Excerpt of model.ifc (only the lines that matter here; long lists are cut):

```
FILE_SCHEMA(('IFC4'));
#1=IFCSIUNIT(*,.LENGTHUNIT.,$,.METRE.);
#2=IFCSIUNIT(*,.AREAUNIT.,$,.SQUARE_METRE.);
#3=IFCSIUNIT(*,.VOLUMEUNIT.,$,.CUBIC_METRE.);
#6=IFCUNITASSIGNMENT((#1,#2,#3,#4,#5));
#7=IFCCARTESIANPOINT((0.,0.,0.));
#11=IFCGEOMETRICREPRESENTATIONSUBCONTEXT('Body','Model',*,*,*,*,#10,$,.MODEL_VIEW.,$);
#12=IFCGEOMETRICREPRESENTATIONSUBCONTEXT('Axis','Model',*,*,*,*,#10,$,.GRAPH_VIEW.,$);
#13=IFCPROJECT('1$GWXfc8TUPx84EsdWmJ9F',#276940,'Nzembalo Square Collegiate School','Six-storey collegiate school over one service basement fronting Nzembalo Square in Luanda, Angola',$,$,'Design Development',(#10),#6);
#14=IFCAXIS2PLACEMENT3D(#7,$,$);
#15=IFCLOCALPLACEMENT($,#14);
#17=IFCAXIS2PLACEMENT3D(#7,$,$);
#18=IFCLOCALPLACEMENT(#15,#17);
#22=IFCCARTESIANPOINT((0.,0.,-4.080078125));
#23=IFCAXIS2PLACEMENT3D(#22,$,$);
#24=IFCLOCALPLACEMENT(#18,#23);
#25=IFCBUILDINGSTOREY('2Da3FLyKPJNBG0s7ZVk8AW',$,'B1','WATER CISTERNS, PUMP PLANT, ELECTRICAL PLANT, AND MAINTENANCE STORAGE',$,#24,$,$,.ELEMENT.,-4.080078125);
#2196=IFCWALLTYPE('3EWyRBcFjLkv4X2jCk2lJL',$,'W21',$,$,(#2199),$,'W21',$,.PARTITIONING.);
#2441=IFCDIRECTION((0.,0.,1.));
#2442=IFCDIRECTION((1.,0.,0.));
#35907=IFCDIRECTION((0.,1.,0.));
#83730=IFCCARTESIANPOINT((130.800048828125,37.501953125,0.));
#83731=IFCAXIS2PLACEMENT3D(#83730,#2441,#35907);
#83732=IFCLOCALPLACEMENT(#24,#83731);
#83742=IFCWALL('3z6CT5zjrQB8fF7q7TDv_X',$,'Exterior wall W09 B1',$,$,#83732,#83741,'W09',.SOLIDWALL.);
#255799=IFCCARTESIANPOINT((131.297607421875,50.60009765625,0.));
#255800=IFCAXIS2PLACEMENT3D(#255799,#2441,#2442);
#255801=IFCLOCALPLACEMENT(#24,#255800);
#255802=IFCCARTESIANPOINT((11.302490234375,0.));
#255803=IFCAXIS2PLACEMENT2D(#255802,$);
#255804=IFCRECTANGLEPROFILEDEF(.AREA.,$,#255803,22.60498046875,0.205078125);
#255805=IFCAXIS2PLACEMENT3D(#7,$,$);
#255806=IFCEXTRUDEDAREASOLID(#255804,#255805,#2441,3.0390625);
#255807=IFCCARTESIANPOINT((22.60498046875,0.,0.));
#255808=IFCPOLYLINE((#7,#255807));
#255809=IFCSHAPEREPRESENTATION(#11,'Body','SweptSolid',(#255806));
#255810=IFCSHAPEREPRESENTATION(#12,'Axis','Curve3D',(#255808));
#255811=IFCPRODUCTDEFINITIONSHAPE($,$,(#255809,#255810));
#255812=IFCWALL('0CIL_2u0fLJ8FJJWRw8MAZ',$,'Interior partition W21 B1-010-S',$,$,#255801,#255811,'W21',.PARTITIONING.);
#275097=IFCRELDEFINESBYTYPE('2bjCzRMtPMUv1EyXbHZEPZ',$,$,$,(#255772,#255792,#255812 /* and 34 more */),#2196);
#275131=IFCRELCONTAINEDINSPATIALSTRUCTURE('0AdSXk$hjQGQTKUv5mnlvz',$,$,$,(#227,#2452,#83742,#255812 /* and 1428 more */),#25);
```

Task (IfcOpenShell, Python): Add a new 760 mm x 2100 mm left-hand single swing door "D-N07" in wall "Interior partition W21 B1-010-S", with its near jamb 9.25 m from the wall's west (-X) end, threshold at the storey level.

```python
import numpy as np
import ifcopenshell
import ifcopenshell.api.feature
import ifcopenshell.api.geometry
import ifcopenshell.api.root
import ifcopenshell.api.spatial
import ifcopenshell.geom
import ifcopenshell.util.element
import ifcopenshell.util.placement
import ifcopenshell.util.representation
import ifcopenshell.util.shape
import ifcopenshell.util.unit

model = ifcopenshell.open("model.ifc")
unit_scale = ifcopenshell.util.unit.calculate_unit_scale(model)
settings = ifcopenshell.geom.settings()


def volume(element):
    """Net volume in cubic metres, openings subtracted."""
    shape = ifcopenshell.geom.create_shape(settings, element)
    return ifcopenshell.util.shape.get_volume(shape.geometry)


wall = model.by_id(255812)
storey = ifcopenshell.util.element.get_container(wall, ifc_class="IfcBuildingStorey")
context = ifcopenshell.util.representation.get_context(model, "Model", "Body", "MODEL_VIEW")
before = volume(wall)

width, height, from_end, sill = 0.76, 2.1, 9.25, 0.0  # metres

# The wall runs along its own X axis, and the end named is its -X end.
wall_shape = ifcopenshell.geom.create_shape(settings, wall)
x, y, z = ifcopenshell.util.shape.get_vertices(wall_shape.geometry).T
start = x.min() + from_end
face, thickness = float(y.min()), float(y.max() - y.min())
wall_matrix = ifcopenshell.util.placement.get_local_placement(wall.ObjectPlacement)
level = ifcopenshell.util.placement.get_local_placement(storey.ObjectPlacement)[2, 3]


def in_wall(x, y):
    """Placement at x, y metres in the wall's axes, at sill height."""
    matrix = wall_matrix.copy()
    matrix[:, 3] = wall_matrix @ np.array([x / unit_scale, y / unit_scale, 0.0, 1.0])
    matrix[2, 3] = level + sill / unit_scale
    return matrix


# Opening: a box that overshoots both wall faces by 50 mm.
opening = ifcopenshell.api.root.create_entity(model, ifc_class="IfcOpeningElement", predefined_type="OPENING")
box = ifcopenshell.api.geometry.add_wall_representation(
    model, context=context, length=width, height=height, thickness=thickness + 0.1
)
ifcopenshell.api.geometry.assign_representation(model, product=opening, representation=box)
ifcopenshell.api.geometry.edit_object_placement(model, product=opening, matrix=in_wall(start, face - 0.05), is_si=False)
ifcopenshell.api.feature.add_feature(model, feature=opening, element=wall)

door = ifcopenshell.api.root.create_entity(model, ifc_class="IfcDoor", name="D-N07", predefined_type="DOOR")
door.OverallWidth, door.OverallHeight = width / unit_scale, height / unit_scale
door.OperationType = "SINGLE_SWING_LEFT"
body = ifcopenshell.api.geometry.add_door_representation(
    model,
    context=context,
    overall_width=door.OverallWidth,
    overall_height=door.OverallHeight,
    operation_type="SINGLE_SWING_LEFT",
    lining_properties={"LiningDepth": thickness / unit_scale, "ThresholdDepth": thickness / unit_scale},
)
ifcopenshell.api.geometry.assign_representation(model, product=door, representation=body)
ifcopenshell.api.spatial.assign_container(model, products=[door], relating_structure=storey)
ifcopenshell.api.feature.add_filling(model, opening=opening, element=door)

# The lining spans the wall, so the door starts at the wall face.
ifcopenshell.api.geometry.edit_object_placement(model, product=door, matrix=in_wall(start, face), is_si=False)

after = volume(wall)

print(f"wall volume {before:.3f} -> {after:.3f} m3")

model.write("model_rev.ifc")
```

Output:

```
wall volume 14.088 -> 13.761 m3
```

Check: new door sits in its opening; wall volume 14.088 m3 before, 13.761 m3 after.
